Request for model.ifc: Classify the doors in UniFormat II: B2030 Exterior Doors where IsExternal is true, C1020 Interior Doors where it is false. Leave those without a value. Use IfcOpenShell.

First a look at what the model holds.

```python
import ifcopenshell
import ifcopenshell.util.element

model = ifcopenshell.open("model.ifc")
print(model.schema)
print("classifications:", [c.Name for c in model.by_type("IfcClassification")])
values = [ifcopenshell.util.element.get_pset(e, "Pset_DoorCommon", "IsExternal") for e in model.by_type("IfcDoor")]
for value in (True, False, None):
    print("IsExternal", value, values.count(value))
```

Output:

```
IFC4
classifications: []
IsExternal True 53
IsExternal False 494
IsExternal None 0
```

```python
import ifcopenshell
import ifcopenshell.api.classification
import ifcopenshell.util.element

model = ifcopenshell.open("model.ifc")

system = ifcopenshell.api.classification.add_classification(model, classification="UniFormat II")

doors = model.by_type("IfcDoor")
external = {e: ifcopenshell.util.element.get_pset(e, "Pset_DoorCommon", "IsExternal") for e in doors}
for flag, code, name in ((True, "B2030", "Exterior Doors"), (False, "C1020", "Interior Doors")):
    products = [e for e in doors if external[e] is flag]
    ifcopenshell.api.classification.add_reference(
        model, products=products, classification=system, identification=code, name=name
    )
    print(code, len(products))

model.write("model-out.ifc")
```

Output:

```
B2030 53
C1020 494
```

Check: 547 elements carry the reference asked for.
